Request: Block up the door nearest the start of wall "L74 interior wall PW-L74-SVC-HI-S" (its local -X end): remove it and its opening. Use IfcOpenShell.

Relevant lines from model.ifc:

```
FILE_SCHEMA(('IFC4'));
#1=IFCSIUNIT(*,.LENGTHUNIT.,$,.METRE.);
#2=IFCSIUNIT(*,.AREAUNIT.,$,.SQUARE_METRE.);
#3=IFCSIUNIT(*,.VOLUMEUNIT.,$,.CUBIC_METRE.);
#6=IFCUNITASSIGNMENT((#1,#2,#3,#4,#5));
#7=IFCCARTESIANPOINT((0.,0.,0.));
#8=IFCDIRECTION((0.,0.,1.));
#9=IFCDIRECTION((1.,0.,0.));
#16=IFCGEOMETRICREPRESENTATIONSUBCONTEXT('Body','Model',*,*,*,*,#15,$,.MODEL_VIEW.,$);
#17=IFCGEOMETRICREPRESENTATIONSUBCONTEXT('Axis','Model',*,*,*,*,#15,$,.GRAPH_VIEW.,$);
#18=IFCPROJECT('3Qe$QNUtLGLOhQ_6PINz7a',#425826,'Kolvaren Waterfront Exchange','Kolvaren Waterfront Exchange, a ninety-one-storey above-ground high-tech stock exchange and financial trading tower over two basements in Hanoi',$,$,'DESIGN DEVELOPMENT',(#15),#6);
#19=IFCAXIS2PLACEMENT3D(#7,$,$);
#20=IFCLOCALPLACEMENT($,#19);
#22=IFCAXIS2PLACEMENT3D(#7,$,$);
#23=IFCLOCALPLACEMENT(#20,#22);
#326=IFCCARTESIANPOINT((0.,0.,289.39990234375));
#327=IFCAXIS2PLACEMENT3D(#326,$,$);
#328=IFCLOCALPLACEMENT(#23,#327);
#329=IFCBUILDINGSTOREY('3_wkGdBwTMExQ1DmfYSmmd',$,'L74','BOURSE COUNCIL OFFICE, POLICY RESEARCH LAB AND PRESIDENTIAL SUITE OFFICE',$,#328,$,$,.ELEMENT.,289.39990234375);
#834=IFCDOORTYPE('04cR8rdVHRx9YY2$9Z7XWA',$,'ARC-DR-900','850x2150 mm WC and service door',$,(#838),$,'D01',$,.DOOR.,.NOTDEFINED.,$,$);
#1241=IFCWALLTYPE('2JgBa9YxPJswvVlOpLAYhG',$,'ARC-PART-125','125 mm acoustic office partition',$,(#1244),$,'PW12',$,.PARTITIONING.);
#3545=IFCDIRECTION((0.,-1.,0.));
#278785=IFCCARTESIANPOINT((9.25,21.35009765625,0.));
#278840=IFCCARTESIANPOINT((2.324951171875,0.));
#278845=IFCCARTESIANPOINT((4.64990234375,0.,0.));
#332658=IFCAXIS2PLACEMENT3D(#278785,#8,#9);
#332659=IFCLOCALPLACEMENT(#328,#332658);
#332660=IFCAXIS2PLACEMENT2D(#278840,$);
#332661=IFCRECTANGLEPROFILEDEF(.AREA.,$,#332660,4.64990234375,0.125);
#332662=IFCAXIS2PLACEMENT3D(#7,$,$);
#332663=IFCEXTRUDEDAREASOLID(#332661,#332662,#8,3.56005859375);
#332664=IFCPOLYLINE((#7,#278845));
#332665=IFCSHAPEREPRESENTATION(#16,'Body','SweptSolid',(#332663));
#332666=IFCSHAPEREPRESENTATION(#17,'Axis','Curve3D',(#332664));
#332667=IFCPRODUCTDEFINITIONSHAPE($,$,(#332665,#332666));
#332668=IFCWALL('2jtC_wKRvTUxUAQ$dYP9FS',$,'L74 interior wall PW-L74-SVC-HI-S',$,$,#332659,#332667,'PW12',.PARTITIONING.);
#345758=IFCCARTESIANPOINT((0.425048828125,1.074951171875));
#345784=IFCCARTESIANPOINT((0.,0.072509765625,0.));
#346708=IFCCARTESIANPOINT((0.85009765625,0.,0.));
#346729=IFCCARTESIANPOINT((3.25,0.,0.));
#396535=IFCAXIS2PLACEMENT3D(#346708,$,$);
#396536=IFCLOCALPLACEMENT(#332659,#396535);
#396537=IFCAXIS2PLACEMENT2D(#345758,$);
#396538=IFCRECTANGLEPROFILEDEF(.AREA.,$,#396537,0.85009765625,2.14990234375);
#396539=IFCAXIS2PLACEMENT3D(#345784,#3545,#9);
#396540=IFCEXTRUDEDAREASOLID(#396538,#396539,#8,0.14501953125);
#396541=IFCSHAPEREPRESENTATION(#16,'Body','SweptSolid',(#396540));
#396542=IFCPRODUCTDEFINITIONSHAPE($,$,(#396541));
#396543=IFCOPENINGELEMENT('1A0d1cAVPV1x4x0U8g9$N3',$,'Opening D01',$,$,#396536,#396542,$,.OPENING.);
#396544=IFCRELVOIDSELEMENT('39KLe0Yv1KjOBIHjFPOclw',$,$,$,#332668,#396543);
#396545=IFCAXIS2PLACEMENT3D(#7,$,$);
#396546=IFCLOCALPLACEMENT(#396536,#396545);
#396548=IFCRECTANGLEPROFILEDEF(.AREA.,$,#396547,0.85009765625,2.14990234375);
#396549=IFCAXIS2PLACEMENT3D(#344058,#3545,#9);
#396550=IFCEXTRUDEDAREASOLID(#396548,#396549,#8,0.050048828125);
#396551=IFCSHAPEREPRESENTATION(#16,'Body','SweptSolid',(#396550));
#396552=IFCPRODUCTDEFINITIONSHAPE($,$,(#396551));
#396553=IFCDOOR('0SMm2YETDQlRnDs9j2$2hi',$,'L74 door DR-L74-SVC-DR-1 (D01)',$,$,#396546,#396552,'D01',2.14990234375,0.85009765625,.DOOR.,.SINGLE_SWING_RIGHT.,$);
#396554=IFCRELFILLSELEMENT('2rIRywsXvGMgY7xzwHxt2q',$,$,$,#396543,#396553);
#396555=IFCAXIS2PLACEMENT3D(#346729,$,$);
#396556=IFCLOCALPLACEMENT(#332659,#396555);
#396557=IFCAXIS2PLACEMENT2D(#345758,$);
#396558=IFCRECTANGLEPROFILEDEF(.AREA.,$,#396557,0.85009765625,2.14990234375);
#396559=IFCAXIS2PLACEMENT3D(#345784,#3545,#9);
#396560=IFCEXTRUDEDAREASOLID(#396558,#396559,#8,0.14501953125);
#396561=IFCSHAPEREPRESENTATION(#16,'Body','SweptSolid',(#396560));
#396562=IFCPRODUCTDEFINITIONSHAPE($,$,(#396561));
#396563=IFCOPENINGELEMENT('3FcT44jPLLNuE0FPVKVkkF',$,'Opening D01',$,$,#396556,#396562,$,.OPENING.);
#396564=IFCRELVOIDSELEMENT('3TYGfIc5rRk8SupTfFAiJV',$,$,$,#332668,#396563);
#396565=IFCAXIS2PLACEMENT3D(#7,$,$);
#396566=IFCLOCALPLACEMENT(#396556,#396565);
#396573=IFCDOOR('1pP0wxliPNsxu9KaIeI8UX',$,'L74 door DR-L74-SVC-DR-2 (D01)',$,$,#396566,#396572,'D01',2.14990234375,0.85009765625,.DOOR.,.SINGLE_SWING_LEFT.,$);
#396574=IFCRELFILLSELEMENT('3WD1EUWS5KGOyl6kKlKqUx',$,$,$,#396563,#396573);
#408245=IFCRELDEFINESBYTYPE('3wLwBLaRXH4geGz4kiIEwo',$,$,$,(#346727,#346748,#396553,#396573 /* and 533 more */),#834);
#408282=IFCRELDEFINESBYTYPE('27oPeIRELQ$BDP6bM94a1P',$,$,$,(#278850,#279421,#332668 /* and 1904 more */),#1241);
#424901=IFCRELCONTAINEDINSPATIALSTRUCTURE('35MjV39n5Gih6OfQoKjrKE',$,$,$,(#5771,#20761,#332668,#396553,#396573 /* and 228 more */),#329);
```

```python
import ifcopenshell
import ifcopenshell.api.feature
import ifcopenshell.api.root
import ifcopenshell.geom
import ifcopenshell.util.shape

model = ifcopenshell.open("model.ifc")
settings = ifcopenshell.geom.settings()


def volume(element):
    """Net volume in cubic metres, openings subtracted."""
    shape = ifcopenshell.geom.create_shape(settings, element)
    return ifcopenshell.util.shape.get_volume(shape.geometry)


door = model.by_guid("0SMm2YETDQlRnDs9j2$2hi")
opening = door.FillsVoids[0].RelatingOpeningElement
wall = opening.VoidsElements[0].RelatingBuildingElement
before = volume(wall)

ifcopenshell.api.root.remove_product(model, product=door)
ifcopenshell.api.feature.remove_feature(model, feature=opening)

after = volume(wall)

print(f"wall volume {before:.3f} -> {after:.3f} m3")

model.write("model-out.ifc")
```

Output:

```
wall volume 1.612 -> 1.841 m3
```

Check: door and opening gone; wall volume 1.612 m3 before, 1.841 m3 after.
